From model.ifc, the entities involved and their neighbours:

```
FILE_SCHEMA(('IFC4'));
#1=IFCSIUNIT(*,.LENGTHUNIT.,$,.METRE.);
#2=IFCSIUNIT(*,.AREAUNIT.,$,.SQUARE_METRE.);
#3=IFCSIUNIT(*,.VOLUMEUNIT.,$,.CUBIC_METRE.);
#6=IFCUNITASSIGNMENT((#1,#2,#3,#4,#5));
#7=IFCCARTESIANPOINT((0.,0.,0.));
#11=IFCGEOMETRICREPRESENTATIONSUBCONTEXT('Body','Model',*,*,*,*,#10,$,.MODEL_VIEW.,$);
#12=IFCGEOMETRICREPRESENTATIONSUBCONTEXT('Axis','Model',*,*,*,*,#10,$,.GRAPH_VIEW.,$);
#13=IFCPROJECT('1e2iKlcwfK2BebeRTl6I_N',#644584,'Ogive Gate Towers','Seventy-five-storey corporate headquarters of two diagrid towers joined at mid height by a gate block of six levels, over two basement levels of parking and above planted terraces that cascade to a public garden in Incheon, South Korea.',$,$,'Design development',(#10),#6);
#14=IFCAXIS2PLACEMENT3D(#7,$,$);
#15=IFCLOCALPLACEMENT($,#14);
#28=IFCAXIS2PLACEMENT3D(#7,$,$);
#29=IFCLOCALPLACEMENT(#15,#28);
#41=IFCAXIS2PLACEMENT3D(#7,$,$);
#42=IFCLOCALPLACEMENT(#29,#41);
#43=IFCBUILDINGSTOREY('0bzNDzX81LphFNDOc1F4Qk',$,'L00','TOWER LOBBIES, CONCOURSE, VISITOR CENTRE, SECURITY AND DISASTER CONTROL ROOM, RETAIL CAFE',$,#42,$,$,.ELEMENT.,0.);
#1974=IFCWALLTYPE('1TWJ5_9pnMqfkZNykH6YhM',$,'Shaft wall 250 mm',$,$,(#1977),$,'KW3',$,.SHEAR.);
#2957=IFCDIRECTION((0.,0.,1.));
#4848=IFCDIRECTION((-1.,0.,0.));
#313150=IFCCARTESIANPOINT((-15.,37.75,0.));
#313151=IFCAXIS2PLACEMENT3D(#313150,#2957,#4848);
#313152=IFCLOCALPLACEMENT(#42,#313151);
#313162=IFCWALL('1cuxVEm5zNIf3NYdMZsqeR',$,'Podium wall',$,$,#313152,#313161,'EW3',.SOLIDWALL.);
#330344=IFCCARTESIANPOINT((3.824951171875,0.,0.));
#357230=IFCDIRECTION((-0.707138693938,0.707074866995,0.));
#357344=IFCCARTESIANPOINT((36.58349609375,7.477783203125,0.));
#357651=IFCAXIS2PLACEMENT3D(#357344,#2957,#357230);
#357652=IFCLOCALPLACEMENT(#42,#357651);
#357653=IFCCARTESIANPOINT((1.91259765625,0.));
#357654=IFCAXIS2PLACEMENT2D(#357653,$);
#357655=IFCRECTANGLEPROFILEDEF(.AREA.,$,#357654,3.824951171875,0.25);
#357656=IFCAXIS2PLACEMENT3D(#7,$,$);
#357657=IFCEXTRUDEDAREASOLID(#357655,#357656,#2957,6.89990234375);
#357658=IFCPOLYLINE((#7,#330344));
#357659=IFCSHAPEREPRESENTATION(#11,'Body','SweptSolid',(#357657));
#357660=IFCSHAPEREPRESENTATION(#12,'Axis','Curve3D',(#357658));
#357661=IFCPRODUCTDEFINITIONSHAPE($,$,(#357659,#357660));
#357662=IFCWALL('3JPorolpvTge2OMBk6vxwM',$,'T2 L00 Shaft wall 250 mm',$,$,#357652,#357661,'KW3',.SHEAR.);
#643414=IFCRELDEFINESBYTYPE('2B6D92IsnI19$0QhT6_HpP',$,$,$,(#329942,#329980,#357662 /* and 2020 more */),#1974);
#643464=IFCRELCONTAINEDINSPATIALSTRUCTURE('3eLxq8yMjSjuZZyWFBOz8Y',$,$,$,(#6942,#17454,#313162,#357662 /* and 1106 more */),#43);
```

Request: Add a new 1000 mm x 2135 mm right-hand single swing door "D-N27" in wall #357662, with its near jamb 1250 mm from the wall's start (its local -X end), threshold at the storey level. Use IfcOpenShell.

```python
import numpy as np
import ifcopenshell
import ifcopenshell.api.feature
import ifcopenshell.api.geometry
import ifcopenshell.api.root
import ifcopenshell.api.spatial
import ifcopenshell.geom
import ifcopenshell.util.element
import ifcopenshell.util.placement
import ifcopenshell.util.representation
import ifcopenshell.util.shape
import ifcopenshell.util.unit

model = ifcopenshell.open("model.ifc")
unit_scale = ifcopenshell.util.unit.calculate_unit_scale(model)
settings = ifcopenshell.geom.settings()


def volume(element):
    """Net volume in cubic metres, openings subtracted."""
    shape = ifcopenshell.geom.create_shape(settings, element)
    return ifcopenshell.util.shape.get_volume(shape.geometry)


wall = model.by_id(357662)
storey = ifcopenshell.util.element.get_container(wall, ifc_class="IfcBuildingStorey")
context = ifcopenshell.util.representation.get_context(model, "Model", "Body", "MODEL_VIEW")
before = volume(wall)

width, height, from_end, sill = 1, 2.135, 1.25, 0.0  # metres

# The wall runs along its own X axis, and the end named is its -X end.
wall_shape = ifcopenshell.geom.create_shape(settings, wall)
x, y, z = ifcopenshell.util.shape.get_vertices(wall_shape.geometry).T
start = x.min() + from_end
face, thickness = float(y.min()), float(y.max() - y.min())
wall_matrix = ifcopenshell.util.placement.get_local_placement(wall.ObjectPlacement)
level = ifcopenshell.util.placement.get_local_placement(storey.ObjectPlacement)[2, 3]


def in_wall(x, y):
    """Placement at x, y metres in the wall's axes, at sill height."""
    matrix = wall_matrix.copy()
    matrix[:, 3] = wall_matrix @ np.array([x / unit_scale, y / unit_scale, 0.0, 1.0])
    matrix[2, 3] = level + sill / unit_scale
    return matrix


# Opening: a box that overshoots both wall faces by 50 mm.
opening = ifcopenshell.api.root.create_entity(model, ifc_class="IfcOpeningElement", predefined_type="OPENING")
box = ifcopenshell.api.geometry.add_wall_representation(
    model, context=context, length=width, height=height, thickness=thickness + 0.1
)
ifcopenshell.api.geometry.assign_representation(model, product=opening, representation=box)
ifcopenshell.api.geometry.edit_object_placement(model, product=opening, matrix=in_wall(start, face - 0.05), is_si=False)
ifcopenshell.api.feature.add_feature(model, feature=opening, element=wall)

door = ifcopenshell.api.root.create_entity(model, ifc_class="IfcDoor", name="D-N27", predefined_type="DOOR")
door.OverallWidth, door.OverallHeight = width / unit_scale, height / unit_scale
door.OperationType = "SINGLE_SWING_RIGHT"
body = ifcopenshell.api.geometry.add_door_representation(
    model,
    context=context,
    overall_width=door.OverallWidth,
    overall_height=door.OverallHeight,
    operation_type="SINGLE_SWING_RIGHT",
    lining_properties={"LiningDepth": thickness / unit_scale, "ThresholdDepth": thickness / unit_scale},
)
ifcopenshell.api.geometry.assign_representation(model, product=door, representation=body)
ifcopenshell.api.spatial.assign_container(model, products=[door], relating_structure=storey)
ifcopenshell.api.feature.add_filling(model, opening=opening, element=door)

# The lining spans the wall, so the door starts at the wall face.
ifcopenshell.api.geometry.edit_object_placement(model, product=door, matrix=in_wall(start, face), is_si=False)

after = volume(wall)

print(f"wall volume {before:.3f} -> {after:.3f} m3")

model.write("model_edited.ifc")
```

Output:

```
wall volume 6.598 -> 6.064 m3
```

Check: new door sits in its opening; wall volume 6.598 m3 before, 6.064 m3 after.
